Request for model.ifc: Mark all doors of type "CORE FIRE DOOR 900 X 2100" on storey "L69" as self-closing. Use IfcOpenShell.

First a look at what the model holds.

```python
import ifcopenshell
import ifcopenshell.util.element

model = ifcopenshell.open("model.ifc")
print(model.schema)
storey = next(s for s in model.by_type("IfcBuildingStorey") if s.Name == "L69")
doors = [e for e in ifcopenshell.util.element.get_decomposition(storey) if e.is_a("IfcDoor")]
seen = {}
for e in doors:
    element_type = ifcopenshell.util.element.get_type(e)
    key = (element_type.Name if element_type != e and element_type else None, ifcopenshell.util.element.get_pset(e, "Pset_DoorCommon", "SelfClosing"))
    seen[key] = seen.get(key, 0) + 1
for (name, value), count in sorted(seen.items(), key=str):
    print(count, "x", name, "|", value)
```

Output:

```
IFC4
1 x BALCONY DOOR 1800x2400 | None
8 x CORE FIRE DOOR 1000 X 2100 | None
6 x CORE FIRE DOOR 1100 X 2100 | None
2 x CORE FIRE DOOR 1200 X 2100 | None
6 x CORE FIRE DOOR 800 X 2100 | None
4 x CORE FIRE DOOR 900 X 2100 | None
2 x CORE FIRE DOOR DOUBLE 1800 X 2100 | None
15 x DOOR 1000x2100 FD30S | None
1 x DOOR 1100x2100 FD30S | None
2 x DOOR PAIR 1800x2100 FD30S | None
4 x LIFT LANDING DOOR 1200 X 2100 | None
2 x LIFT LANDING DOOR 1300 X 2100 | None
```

```python
import ifcopenshell
import ifcopenshell.api.pset
import ifcopenshell.util.element

model = ifcopenshell.open("model.ifc")

storey = next(s for s in model.by_type("IfcBuildingStorey") if s.Name == "L69")
doors = [e for e in ifcopenshell.util.element.get_decomposition(storey) if e.is_a("IfcDoor")]

count = 0
for e in doors:
    element_type = ifcopenshell.util.element.get_type(e)
    if element_type in (None, e) or element_type.Name != "CORE FIRE DOOR 900 X 2100":
        continue
    found = ifcopenshell.util.element.get_pset(e, "Pset_DoorCommon", should_inherit=False)
    if found:
        pset = model.by_id(found["id"])
        if len(ifcopenshell.util.element.get_elements_by_pset(pset)) > 1:
            pset = ifcopenshell.api.pset.unshare_pset(model, products=[e], pset=pset)[0]
    else:
        pset = ifcopenshell.api.pset.add_pset(model, product=e, name="Pset_DoorCommon")
    ifcopenshell.api.pset.edit_pset(model, pset=pset, properties={"SelfClosing": True})
    count += 1

print(count, "doors updated")

model.write("model-out.ifc")
```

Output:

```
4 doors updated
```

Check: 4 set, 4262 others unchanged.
